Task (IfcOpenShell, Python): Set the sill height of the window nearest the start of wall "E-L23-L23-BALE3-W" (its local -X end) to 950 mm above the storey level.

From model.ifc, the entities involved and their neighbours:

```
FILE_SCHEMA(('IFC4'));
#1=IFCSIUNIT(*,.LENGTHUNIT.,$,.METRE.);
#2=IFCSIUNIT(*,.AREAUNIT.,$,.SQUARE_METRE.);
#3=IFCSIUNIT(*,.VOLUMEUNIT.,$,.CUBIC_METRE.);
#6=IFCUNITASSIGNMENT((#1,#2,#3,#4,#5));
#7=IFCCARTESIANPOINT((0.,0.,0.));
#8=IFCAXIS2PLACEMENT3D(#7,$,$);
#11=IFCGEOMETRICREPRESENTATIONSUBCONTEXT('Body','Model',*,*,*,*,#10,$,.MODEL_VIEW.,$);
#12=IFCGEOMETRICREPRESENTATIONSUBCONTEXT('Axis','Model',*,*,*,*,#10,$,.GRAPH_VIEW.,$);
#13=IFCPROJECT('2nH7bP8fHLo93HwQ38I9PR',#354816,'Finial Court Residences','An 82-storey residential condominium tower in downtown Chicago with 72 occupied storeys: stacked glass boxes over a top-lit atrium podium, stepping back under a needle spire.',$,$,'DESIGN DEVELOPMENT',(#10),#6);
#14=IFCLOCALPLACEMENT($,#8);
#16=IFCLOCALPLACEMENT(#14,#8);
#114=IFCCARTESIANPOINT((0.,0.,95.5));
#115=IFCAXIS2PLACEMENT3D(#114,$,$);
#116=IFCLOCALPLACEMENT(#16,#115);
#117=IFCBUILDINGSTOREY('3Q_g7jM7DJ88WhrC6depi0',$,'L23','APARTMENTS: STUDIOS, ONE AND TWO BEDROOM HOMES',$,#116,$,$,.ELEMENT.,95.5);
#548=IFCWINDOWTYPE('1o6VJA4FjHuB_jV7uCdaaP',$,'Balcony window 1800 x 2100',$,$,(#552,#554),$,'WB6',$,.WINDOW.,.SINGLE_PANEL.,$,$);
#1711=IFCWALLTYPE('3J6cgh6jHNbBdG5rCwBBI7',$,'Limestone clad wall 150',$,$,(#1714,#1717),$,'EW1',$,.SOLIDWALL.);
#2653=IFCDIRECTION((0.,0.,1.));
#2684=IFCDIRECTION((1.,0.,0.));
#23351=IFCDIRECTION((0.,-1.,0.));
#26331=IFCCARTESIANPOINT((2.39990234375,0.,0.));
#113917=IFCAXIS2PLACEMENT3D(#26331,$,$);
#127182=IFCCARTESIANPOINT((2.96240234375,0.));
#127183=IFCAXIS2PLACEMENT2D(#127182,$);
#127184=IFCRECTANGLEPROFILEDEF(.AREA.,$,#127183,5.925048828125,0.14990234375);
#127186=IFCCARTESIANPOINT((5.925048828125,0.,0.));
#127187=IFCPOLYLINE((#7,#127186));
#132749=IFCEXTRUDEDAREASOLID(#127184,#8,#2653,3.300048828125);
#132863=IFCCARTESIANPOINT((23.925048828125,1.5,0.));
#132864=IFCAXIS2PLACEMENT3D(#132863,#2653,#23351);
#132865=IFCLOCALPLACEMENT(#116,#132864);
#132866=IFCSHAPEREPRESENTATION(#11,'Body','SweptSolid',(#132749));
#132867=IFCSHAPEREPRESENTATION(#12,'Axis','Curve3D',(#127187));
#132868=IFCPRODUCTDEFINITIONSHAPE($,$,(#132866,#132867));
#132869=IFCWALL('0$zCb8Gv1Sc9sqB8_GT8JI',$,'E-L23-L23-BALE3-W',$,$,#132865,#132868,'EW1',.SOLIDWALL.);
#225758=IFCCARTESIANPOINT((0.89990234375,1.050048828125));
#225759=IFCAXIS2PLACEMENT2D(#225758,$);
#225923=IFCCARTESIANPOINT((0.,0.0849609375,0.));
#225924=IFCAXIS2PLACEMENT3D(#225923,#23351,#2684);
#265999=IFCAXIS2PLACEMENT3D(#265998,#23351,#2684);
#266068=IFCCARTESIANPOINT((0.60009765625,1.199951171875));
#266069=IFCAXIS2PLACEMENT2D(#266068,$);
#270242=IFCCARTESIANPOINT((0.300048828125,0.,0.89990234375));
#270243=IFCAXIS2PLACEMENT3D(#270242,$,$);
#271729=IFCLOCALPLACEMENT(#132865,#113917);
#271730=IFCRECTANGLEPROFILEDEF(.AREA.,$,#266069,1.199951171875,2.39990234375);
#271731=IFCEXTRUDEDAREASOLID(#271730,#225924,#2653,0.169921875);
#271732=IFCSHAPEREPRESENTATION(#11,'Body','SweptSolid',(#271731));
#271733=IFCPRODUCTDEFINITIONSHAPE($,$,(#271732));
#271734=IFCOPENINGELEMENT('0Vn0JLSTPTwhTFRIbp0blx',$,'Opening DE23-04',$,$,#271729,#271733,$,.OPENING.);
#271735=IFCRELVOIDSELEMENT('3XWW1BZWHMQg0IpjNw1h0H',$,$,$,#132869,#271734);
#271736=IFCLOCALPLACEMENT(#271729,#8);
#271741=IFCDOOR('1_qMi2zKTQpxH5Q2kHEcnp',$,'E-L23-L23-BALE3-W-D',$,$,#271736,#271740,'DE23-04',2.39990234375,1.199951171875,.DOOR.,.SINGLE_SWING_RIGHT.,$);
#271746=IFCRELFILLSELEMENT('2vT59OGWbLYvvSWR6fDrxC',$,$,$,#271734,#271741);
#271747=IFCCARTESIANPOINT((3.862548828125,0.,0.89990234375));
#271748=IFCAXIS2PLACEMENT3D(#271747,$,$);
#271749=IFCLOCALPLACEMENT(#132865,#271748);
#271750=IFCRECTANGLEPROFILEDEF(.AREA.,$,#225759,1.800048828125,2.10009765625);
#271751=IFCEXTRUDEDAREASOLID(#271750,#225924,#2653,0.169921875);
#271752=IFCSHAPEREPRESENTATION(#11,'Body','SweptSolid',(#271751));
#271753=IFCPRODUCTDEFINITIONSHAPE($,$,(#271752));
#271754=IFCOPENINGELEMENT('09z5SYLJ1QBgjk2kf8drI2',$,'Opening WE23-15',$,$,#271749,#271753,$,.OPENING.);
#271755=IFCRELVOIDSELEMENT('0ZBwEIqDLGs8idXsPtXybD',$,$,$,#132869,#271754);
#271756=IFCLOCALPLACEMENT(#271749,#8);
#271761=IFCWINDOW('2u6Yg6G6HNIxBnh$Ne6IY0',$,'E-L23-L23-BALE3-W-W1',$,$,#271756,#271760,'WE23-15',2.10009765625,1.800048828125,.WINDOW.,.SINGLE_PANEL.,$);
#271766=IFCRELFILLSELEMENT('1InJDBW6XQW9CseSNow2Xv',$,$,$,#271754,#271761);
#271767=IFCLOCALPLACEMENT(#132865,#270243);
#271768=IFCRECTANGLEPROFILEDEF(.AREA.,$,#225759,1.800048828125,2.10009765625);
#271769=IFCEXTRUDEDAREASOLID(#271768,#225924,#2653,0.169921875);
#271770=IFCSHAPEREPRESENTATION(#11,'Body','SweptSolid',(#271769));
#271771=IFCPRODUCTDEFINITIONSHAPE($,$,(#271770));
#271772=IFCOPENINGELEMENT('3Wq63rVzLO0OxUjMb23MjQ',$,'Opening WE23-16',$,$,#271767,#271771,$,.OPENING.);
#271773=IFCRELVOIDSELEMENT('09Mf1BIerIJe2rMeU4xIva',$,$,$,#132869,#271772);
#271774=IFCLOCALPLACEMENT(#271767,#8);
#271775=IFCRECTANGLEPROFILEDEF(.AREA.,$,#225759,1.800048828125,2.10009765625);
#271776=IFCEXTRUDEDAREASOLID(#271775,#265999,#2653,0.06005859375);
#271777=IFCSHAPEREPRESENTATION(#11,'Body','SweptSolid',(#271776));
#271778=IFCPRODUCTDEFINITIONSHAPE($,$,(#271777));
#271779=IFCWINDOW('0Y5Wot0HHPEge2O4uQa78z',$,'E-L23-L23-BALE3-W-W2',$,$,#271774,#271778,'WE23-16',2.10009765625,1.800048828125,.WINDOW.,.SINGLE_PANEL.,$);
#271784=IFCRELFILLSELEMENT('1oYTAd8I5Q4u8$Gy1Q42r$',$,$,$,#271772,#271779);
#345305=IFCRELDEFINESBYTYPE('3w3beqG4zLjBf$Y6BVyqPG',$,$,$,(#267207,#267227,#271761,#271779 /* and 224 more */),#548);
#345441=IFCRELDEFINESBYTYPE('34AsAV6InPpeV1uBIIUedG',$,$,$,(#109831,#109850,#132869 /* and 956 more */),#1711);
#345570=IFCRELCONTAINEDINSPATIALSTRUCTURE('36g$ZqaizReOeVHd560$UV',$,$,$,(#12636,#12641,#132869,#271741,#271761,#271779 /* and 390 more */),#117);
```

```python
import numpy as np
import ifcopenshell
import ifcopenshell.api.geometry
import ifcopenshell.geom
import ifcopenshell.util.element
import ifcopenshell.util.placement
import ifcopenshell.util.shape
import ifcopenshell.util.unit

model = ifcopenshell.open("model.ifc")
unit_scale = ifcopenshell.util.unit.calculate_unit_scale(model)

window = model.by_guid("0Y5Wot0HHPEge2O4uQa78z")
opening = window.FillsVoids[0].RelatingOpeningElement
storey = ifcopenshell.util.element.get_container(window, ifc_class="IfcBuildingStorey")
level = ifcopenshell.util.placement.get_local_placement(storey.ObjectPlacement)[2, 3]

# The opening's origin need not be at the sill, so measure its lowest point.
shape = ifcopenshell.geom.create_shape(ifcopenshell.geom.settings(), opening)
bottom = ifcopenshell.util.shape.get_shape_bottom_elevation(shape, shape.geometry) / unit_scale
dz = level + 0.95 / unit_scale - bottom

shift = np.array([0.0, 0.0, dz])
# The window is placed relative to its opening, so it follows when the opening moves.
matrix = ifcopenshell.util.placement.get_local_placement(opening.ObjectPlacement)
matrix[:3, 3] += shift
ifcopenshell.api.geometry.edit_object_placement(
    model, product=opening, matrix=matrix, is_si=False, should_transform_children=True
)

print(f"moved by {dz * unit_scale:+.3f} m")

model.write("model_updated.ifc")
```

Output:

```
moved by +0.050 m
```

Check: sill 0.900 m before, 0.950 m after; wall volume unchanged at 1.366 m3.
